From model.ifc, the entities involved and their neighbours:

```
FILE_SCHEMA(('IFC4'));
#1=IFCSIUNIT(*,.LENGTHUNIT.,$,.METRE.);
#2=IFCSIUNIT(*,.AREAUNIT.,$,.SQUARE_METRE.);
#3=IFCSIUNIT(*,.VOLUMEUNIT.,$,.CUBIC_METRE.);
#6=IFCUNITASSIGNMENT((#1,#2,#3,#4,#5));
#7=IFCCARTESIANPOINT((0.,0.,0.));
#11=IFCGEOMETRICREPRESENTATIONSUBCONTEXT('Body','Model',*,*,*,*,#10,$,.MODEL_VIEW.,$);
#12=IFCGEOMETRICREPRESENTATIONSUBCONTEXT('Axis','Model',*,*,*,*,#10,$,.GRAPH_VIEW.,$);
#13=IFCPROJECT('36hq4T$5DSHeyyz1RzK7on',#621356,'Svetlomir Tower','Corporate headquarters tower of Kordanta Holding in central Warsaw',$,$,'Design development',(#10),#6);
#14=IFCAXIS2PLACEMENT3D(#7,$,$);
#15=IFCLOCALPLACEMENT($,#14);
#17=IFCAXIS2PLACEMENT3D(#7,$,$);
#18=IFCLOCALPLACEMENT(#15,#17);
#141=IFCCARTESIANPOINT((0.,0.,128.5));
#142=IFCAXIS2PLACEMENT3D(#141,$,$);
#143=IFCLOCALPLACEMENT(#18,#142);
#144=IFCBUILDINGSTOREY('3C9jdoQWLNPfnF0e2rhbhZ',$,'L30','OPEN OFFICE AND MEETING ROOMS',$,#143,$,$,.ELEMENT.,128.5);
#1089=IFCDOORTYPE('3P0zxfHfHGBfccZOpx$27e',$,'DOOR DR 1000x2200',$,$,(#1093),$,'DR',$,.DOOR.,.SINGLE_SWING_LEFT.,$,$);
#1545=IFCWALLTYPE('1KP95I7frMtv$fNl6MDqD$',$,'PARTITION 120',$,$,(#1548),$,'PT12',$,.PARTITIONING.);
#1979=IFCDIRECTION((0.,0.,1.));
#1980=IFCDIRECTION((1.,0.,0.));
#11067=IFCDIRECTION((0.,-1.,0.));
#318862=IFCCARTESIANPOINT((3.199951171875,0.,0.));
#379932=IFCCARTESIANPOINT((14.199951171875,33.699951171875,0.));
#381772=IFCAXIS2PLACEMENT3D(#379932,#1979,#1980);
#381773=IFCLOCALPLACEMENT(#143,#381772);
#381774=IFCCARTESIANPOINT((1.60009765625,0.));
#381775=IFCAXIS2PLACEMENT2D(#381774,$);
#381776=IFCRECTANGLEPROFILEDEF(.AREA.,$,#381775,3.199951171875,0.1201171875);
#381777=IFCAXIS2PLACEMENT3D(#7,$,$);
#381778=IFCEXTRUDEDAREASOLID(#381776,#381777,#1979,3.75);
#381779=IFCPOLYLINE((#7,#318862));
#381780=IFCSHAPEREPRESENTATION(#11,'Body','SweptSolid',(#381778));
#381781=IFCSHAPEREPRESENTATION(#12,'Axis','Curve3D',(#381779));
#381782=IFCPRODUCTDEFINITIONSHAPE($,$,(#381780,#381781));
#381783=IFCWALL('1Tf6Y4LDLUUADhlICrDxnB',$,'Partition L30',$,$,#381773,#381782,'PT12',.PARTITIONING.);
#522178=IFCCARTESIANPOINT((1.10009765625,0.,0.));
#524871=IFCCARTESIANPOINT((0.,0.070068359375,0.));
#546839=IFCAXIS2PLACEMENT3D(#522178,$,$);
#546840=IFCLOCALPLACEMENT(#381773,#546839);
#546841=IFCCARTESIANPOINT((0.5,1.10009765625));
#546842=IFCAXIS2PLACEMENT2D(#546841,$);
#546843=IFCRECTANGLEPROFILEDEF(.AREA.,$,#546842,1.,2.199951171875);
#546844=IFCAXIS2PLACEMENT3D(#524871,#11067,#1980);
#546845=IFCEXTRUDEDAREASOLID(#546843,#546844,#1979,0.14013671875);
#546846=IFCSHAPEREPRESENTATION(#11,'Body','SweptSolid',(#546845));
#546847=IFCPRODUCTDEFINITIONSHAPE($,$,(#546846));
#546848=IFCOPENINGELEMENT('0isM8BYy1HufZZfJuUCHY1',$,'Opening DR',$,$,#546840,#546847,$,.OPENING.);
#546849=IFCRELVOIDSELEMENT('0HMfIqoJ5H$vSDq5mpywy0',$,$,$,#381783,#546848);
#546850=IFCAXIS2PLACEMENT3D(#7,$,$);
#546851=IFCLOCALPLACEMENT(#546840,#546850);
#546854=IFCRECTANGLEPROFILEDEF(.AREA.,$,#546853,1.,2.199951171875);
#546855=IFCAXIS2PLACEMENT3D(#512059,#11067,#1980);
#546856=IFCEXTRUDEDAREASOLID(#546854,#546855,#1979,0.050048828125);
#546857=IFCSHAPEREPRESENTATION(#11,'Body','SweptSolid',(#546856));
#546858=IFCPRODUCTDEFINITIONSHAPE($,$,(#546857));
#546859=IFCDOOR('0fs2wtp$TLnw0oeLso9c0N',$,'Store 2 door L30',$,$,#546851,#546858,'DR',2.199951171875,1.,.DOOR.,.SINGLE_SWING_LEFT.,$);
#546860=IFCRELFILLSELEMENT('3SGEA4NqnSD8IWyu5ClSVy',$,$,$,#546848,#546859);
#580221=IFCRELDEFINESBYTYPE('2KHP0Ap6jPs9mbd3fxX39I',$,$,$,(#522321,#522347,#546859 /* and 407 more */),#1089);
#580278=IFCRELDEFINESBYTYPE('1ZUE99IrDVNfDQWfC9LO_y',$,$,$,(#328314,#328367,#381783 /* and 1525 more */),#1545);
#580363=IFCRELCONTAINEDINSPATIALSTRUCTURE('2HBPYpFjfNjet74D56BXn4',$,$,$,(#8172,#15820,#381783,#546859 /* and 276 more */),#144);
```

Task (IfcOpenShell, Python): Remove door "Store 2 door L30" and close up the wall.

```python
import ifcopenshell
import ifcopenshell.api.feature
import ifcopenshell.api.root
import ifcopenshell.geom
import ifcopenshell.util.shape

model = ifcopenshell.open("model.ifc")
settings = ifcopenshell.geom.settings()


def volume(element):
    """Net volume in cubic metres, openings subtracted."""
    shape = ifcopenshell.geom.create_shape(settings, element)
    return ifcopenshell.util.shape.get_volume(shape.geometry)


door = model.by_guid("0fs2wtp$TLnw0oeLso9c0N")
opening = door.FillsVoids[0].RelatingOpeningElement
wall = opening.VoidsElements[0].RelatingBuildingElement
before = volume(wall)

ifcopenshell.api.root.remove_product(model, product=door)
ifcopenshell.api.feature.remove_feature(model, feature=opening)

after = volume(wall)

print(f"wall volume {before:.3f} -> {after:.3f} m3")

model.write("model_updated.ifc")
```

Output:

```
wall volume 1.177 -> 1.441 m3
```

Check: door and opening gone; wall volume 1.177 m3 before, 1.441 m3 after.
